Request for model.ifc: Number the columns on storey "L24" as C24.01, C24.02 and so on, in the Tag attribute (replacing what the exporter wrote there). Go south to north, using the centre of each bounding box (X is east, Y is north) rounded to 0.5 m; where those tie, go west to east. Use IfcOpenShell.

First a look at what the model holds.

```python
import ifcopenshell
import ifcopenshell.util.element
import ifcopenshell.util.placement

model = ifcopenshell.open("model.ifc")
print(model.schema)
storey = next(s for s in model.by_type("IfcBuildingStorey") if s.Name == "L24")
columns = [e for e in ifcopenshell.util.element.get_decomposition(storey) if e.is_a("IfcColumn")]
for e in sorted(columns, key=lambda e: e.id()):
    origin = ifcopenshell.util.placement.get_local_placement(e.ObjectPlacement)[:3, 3]
    print(e.id(), e.Tag, e.Name, origin.round(2) + 0.0, sep=" | ")
```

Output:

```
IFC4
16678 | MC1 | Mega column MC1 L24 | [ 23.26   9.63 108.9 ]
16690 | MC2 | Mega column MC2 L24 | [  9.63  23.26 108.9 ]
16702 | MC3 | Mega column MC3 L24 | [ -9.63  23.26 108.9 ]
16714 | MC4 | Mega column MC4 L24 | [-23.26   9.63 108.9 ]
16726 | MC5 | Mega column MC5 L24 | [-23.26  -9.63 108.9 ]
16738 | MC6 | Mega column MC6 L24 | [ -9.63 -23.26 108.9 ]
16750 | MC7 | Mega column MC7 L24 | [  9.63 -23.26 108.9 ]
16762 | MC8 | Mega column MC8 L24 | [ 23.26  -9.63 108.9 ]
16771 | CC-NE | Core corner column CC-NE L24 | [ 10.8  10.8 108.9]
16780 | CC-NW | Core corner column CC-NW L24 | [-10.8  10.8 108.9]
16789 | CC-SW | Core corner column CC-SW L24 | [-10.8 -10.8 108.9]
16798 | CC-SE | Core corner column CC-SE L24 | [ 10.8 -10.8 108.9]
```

```python
import ifcopenshell
import ifcopenshell.geom
import ifcopenshell.util.element
import ifcopenshell.util.shape

model = ifcopenshell.open("model.ifc")
settings = ifcopenshell.geom.settings()
settings.set("use-world-coords", True)


def centre(element):
    shape = ifcopenshell.geom.create_shape(settings, element)
    return ifcopenshell.util.shape.get_bbox_centroid(shape.geometry)


storey = next(s for s in model.by_type("IfcBuildingStorey") if s.Name == "L24")
columns = [e for e in ifcopenshell.util.element.get_decomposition(storey) if e.is_a("IfcColumn")]

# Insertion points can sit at a corner or the storey origin, so sort by the geometry (in metres).
centres = {e: centre(e) for e in columns}
columns.sort(key=lambda e: (round(centres[e][1] / 0.5), centres[e][0]))

for i, e in enumerate(columns, start=1):
    number = f"C24.{i:02d}"
    e.Tag = number
    print(e.id(), number)

model.write("model_v2.ifc")
```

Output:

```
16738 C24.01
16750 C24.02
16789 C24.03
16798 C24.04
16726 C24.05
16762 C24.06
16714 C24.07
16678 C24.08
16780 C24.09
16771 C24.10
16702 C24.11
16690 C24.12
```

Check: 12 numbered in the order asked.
